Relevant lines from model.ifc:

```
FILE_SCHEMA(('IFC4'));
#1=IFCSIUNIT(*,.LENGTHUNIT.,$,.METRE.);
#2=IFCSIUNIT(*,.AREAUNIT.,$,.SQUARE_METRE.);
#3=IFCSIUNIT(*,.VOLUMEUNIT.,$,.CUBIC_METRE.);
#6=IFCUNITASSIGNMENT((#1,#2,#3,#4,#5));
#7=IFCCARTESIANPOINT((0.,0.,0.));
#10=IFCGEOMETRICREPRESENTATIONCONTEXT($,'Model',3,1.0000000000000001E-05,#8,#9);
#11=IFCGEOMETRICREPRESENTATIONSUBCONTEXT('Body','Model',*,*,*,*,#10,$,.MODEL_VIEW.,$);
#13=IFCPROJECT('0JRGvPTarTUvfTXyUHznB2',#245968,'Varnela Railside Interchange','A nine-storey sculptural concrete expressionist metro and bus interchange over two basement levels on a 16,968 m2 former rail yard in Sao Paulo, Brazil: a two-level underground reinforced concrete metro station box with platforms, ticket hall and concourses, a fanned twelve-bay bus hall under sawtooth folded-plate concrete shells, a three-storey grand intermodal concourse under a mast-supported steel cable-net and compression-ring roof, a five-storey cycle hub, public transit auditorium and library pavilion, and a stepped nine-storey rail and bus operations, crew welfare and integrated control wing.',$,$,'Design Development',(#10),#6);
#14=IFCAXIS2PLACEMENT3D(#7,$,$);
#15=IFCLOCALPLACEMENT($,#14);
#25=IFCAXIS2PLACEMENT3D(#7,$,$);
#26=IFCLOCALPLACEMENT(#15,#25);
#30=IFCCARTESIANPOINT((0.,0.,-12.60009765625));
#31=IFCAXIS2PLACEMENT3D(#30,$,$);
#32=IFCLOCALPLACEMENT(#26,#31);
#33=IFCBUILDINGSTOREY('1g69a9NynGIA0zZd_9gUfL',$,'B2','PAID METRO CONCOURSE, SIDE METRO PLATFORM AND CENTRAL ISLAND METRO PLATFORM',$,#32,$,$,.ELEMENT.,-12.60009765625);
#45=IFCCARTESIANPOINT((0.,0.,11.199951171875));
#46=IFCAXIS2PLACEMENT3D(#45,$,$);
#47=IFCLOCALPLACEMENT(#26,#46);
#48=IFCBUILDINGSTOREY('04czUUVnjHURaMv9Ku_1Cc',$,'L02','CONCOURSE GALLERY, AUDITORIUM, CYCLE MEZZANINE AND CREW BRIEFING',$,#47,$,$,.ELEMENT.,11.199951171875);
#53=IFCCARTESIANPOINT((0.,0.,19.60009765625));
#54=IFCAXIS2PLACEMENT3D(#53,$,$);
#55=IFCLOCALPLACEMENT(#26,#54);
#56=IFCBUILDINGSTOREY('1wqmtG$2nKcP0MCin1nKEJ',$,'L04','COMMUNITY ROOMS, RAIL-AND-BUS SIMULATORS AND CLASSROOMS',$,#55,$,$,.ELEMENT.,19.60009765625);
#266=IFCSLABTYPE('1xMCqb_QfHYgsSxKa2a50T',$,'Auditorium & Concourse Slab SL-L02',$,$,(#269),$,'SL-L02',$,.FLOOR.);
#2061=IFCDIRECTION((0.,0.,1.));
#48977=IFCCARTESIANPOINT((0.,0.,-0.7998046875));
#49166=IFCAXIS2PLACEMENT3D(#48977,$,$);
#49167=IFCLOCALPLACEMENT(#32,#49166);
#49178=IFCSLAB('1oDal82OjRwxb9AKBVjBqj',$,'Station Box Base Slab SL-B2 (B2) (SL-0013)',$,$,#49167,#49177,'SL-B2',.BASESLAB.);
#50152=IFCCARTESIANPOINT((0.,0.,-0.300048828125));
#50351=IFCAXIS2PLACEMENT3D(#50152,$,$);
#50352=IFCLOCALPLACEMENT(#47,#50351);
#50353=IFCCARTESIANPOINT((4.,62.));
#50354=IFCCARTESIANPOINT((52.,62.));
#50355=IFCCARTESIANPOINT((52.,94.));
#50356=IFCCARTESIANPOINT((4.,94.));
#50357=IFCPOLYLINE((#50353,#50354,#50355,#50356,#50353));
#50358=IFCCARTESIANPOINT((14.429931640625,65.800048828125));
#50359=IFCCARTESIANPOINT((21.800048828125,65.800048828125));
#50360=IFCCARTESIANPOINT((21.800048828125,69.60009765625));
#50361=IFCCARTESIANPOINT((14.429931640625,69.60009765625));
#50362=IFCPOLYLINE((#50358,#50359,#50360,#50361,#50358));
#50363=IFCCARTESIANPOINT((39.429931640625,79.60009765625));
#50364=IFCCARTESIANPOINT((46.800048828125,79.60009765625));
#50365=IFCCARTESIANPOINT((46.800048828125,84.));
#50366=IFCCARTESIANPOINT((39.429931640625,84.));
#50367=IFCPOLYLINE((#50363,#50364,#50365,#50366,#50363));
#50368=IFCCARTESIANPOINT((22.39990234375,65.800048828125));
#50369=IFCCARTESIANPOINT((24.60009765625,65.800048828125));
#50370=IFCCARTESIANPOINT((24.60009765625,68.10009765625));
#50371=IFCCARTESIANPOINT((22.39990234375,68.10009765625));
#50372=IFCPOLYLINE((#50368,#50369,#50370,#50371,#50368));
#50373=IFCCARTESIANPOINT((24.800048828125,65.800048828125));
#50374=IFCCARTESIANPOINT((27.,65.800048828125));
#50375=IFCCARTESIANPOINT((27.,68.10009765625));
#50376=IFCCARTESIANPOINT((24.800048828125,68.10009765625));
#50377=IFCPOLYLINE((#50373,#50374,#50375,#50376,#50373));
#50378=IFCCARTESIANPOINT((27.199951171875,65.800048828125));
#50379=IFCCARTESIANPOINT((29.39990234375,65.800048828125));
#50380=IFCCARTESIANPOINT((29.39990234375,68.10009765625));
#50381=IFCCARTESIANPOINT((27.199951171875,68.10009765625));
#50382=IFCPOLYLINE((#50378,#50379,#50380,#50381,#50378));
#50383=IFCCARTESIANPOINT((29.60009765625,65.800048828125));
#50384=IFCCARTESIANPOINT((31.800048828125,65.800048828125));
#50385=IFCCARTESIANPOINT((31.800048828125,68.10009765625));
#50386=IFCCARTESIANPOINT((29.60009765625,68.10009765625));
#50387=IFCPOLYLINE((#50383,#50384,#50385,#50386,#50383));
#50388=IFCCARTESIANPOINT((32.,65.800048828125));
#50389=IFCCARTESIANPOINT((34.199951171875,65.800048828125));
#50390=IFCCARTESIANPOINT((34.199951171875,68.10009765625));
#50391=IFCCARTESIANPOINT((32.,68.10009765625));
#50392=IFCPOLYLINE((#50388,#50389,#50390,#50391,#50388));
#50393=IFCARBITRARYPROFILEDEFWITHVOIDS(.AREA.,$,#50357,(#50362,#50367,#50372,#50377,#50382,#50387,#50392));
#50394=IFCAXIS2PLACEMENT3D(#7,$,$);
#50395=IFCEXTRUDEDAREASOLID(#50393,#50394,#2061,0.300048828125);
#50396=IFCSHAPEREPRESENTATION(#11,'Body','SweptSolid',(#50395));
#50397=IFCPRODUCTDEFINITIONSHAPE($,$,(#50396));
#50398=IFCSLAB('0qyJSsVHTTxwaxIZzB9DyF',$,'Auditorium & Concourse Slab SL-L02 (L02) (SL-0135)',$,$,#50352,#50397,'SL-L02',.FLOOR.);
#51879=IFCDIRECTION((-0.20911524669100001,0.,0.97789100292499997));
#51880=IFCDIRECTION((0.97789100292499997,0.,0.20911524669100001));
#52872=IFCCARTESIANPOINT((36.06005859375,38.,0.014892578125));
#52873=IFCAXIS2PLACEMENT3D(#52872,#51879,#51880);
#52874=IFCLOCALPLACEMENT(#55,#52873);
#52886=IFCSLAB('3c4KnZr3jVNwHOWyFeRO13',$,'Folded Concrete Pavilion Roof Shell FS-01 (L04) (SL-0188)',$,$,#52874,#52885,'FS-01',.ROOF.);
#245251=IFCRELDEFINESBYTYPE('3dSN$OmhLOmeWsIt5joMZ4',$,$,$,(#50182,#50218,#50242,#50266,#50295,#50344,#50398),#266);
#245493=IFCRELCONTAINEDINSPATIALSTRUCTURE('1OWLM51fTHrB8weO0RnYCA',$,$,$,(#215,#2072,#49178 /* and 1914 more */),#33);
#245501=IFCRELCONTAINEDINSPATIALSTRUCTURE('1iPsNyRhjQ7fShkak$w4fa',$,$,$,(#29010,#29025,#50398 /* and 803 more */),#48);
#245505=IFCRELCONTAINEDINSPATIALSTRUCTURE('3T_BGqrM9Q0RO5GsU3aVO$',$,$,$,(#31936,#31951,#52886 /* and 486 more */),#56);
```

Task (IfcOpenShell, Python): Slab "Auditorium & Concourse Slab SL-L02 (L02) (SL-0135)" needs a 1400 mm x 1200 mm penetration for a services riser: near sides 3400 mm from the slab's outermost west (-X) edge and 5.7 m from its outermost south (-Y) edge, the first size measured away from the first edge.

```python
import numpy as np
import ifcopenshell
import ifcopenshell.api.feature
import ifcopenshell.api.geometry
import ifcopenshell.api.root
import ifcopenshell.geom
import ifcopenshell.util.placement
import ifcopenshell.util.representation
import ifcopenshell.util.shape
import ifcopenshell.util.unit

model = ifcopenshell.open("model.ifc")
unit_scale = ifcopenshell.util.unit.calculate_unit_scale(model)
settings = ifcopenshell.geom.settings()


def volume(element):
    """Net volume in cubic metres, openings subtracted."""
    shape = ifcopenshell.geom.create_shape(settings, element)
    return ifcopenshell.util.shape.get_volume(shape.geometry)


slab = model.by_guid("0qyJSsVHTTxwaxIZzB9DyF")
before = volume(slab)

# Extent in the slab's own axes, in metres. The edges named are its -X and -Y sides.
slab_shape = ifcopenshell.geom.create_shape(settings, slab)
vertices = ifcopenshell.util.shape.get_vertices(slab_shape.geometry)
x_min, y_min, bottom = vertices.min(axis=0)
top = vertices[:, 2].max()

opening = ifcopenshell.api.root.create_entity(model, ifc_class="IfcOpeningElement", name="Services riser opening", predefined_type="OPENING")
context = ifcopenshell.util.representation.get_context(model, "Model", "Body", "MODEL_VIEW")
width, depth = 1.4, 1.2
outline = [(0.0, 0.0), (width, 0.0), (width, depth), (0.0, depth), (0.0, 0.0)]
# Overshoot both faces by 50 mm so the cut is clean.
shape = ifcopenshell.api.geometry.add_slab_representation(
    model, context=context, depth=top - bottom + 0.1, polyline=outline
)
ifcopenshell.api.geometry.assign_representation(model, product=opening, representation=shape)

matrix = ifcopenshell.util.placement.get_local_placement(slab.ObjectPlacement)
matrix[:, 3] = matrix @ np.append(np.array([x_min + 3.4, y_min + 5.7, bottom - 0.05]) / unit_scale, 1.0)
ifcopenshell.api.geometry.edit_object_placement(model, product=opening, matrix=matrix, is_si=False)
ifcopenshell.api.feature.add_feature(model, feature=opening, element=slab)

after = volume(slab)

print(f"slab volume {before:.3f} -> {after:.3f} m3")

model.write("model-out.ifc")
```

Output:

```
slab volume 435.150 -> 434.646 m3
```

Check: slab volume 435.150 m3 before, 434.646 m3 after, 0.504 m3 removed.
